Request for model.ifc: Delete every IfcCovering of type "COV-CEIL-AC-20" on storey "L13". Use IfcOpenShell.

First a look at what the model holds.

```python
import ifcopenshell
import ifcopenshell.util.element

model = ifcopenshell.open("model.ifc")
print(model.schema)
storey = next(s for s in model.by_type("IfcBuildingStorey") if s.Name == "L13")
coverings = [e for e in ifcopenshell.util.element.get_decomposition(storey) if e.is_a("IfcCovering")]
seen = {}
for e in coverings:
    element_type = ifcopenshell.util.element.get_type(e)
    name = element_type.Name if element_type not in (None, e) else None
    seen[name] = seen.get(name, 0) + 1
for name, count in sorted(seen.items(), key=str):
    print(count, "x", name)
```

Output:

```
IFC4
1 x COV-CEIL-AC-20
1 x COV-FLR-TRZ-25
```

```python
import ifcopenshell
import ifcopenshell.api.root
import ifcopenshell.util.element

model = ifcopenshell.open("model.ifc")

storey = next(s for s in model.by_type("IfcBuildingStorey") if s.Name == "L13")
coverings = [e for e in ifcopenshell.util.element.get_decomposition(storey) if e.is_a("IfcCovering")]
targets = [e for e in coverings if (t := ifcopenshell.util.element.get_type(e)) not in (None, e) and t.Name == "COV-CEIL-AC-20"]

for e in targets:
    ifcopenshell.api.root.remove_product(model, product=e)
print(len(targets), "removed")

model.write("model_updated.ifc")
```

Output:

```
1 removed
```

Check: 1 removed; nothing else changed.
